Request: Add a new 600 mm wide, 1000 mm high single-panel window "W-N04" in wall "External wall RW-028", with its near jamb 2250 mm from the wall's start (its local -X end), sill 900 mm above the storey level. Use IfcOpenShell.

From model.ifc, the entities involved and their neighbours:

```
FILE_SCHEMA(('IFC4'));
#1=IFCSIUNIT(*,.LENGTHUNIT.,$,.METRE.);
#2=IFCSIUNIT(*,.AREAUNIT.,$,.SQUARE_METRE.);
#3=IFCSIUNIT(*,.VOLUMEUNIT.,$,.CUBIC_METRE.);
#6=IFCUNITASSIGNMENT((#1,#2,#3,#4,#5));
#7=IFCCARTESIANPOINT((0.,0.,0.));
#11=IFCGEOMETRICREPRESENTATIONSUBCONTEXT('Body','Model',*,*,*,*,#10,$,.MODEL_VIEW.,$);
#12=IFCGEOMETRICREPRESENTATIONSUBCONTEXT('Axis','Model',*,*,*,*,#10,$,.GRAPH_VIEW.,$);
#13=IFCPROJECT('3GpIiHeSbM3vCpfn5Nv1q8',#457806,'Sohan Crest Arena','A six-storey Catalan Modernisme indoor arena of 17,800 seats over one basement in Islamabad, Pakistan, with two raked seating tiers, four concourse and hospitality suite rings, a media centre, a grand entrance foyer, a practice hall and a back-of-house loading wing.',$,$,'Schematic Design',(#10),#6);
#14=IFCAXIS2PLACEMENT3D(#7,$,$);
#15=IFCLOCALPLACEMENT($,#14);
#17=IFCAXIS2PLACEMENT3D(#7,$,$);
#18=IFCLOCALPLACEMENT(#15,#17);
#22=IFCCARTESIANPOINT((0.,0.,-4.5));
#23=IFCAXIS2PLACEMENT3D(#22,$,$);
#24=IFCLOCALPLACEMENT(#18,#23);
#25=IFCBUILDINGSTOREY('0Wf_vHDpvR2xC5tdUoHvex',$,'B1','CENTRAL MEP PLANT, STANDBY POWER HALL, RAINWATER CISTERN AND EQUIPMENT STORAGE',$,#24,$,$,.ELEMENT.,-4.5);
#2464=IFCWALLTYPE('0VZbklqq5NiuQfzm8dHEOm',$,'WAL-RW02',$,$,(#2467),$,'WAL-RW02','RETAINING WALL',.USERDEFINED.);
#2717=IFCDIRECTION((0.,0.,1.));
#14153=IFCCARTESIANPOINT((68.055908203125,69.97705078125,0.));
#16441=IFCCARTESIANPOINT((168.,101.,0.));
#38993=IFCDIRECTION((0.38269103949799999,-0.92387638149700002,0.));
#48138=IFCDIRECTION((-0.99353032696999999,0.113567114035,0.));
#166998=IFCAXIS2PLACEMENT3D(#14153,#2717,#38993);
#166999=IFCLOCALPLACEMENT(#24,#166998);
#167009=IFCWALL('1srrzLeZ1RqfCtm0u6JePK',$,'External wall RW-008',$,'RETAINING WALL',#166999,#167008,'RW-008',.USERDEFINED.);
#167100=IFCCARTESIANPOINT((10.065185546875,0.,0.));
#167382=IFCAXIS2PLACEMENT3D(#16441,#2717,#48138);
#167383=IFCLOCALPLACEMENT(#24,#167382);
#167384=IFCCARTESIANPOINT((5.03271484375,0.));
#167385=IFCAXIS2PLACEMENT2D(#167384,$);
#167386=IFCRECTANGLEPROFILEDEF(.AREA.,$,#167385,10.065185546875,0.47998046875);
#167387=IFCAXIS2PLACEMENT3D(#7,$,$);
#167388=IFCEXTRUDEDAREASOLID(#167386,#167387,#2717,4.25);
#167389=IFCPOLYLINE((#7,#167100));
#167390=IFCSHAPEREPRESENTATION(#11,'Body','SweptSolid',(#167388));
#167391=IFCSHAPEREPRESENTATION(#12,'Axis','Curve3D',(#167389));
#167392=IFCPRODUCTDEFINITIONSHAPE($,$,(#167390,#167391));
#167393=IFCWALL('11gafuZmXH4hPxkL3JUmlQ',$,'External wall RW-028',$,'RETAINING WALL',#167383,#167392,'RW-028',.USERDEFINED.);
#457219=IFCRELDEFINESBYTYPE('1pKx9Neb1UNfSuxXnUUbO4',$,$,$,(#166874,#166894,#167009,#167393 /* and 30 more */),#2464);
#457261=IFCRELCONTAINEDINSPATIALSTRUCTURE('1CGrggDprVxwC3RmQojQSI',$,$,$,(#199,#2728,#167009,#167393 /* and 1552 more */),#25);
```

```python
import numpy as np
import ifcopenshell
import ifcopenshell.api.feature
import ifcopenshell.api.geometry
import ifcopenshell.api.root
import ifcopenshell.api.spatial
import ifcopenshell.geom
import ifcopenshell.util.element
import ifcopenshell.util.placement
import ifcopenshell.util.representation
import ifcopenshell.util.shape
import ifcopenshell.util.unit

model = ifcopenshell.open("model.ifc")
unit_scale = ifcopenshell.util.unit.calculate_unit_scale(model)
settings = ifcopenshell.geom.settings()


def volume(element):
    """Net volume in cubic metres, openings subtracted."""
    shape = ifcopenshell.geom.create_shape(settings, element)
    return ifcopenshell.util.shape.get_volume(shape.geometry)


wall = model.by_guid("11gafuZmXH4hPxkL3JUmlQ")
storey = ifcopenshell.util.element.get_container(wall, ifc_class="IfcBuildingStorey")
context = ifcopenshell.util.representation.get_context(model, "Model", "Body", "MODEL_VIEW")
before = volume(wall)

width, height, from_end, sill = 0.6, 1, 2.25, 0.9  # metres

# The wall runs along its own X axis, and the end named is its -X end.
wall_shape = ifcopenshell.geom.create_shape(settings, wall)
x, y, z = ifcopenshell.util.shape.get_vertices(wall_shape.geometry).T
start = x.min() + from_end
face, thickness = float(y.min()), float(y.max() - y.min())
wall_matrix = ifcopenshell.util.placement.get_local_placement(wall.ObjectPlacement)
level = ifcopenshell.util.placement.get_local_placement(storey.ObjectPlacement)[2, 3]


def in_wall(x, y):
    """Placement at x, y metres in the wall's axes, at sill height."""
    matrix = wall_matrix.copy()
    matrix[:, 3] = wall_matrix @ np.array([x / unit_scale, y / unit_scale, 0.0, 1.0])
    matrix[2, 3] = level + sill / unit_scale
    return matrix


# Opening: a box that overshoots both wall faces by 50 mm.
opening = ifcopenshell.api.root.create_entity(model, ifc_class="IfcOpeningElement", predefined_type="OPENING")
box = ifcopenshell.api.geometry.add_wall_representation(
    model, context=context, length=width, height=height, thickness=thickness + 0.1
)
ifcopenshell.api.geometry.assign_representation(model, product=opening, representation=box)
ifcopenshell.api.geometry.edit_object_placement(model, product=opening, matrix=in_wall(start, face - 0.05), is_si=False)
ifcopenshell.api.feature.add_feature(model, feature=opening, element=wall)

window = ifcopenshell.api.root.create_entity(model, ifc_class="IfcWindow", name="W-N04", predefined_type="WINDOW")
window.OverallWidth, window.OverallHeight = width / unit_scale, height / unit_scale
window.PartitioningType = "SINGLE_PANEL"
body = ifcopenshell.api.geometry.add_window_representation(
    model,
    context=context,
    overall_width=window.OverallWidth,
    overall_height=window.OverallHeight,
    partition_type="SINGLE_PANEL",
)
ifcopenshell.api.geometry.assign_representation(model, product=window, representation=body)
ifcopenshell.api.spatial.assign_container(model, products=[window], relating_structure=storey)
ifcopenshell.api.feature.add_filling(model, opening=opening, element=window)

# Centre the window in the wall's thickness.
ifcopenshell.api.geometry.edit_object_placement(model, product=window, matrix=in_wall(start, face), is_si=False)
window_shape = ifcopenshell.geom.create_shape(settings, window)
depth = ifcopenshell.util.shape.get_vertices(window_shape.geometry)[:, 1]
offset = face + thickness / 2 - (depth.min() + depth.max()) / 2
ifcopenshell.api.geometry.edit_object_placement(model, product=window, matrix=in_wall(start, offset), is_si=False)

after = volume(wall)

print(f"wall volume {before:.3f} -> {after:.3f} m3")

model.write("model_v2.ifc")
```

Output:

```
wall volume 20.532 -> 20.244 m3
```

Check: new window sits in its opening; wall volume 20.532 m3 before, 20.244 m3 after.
